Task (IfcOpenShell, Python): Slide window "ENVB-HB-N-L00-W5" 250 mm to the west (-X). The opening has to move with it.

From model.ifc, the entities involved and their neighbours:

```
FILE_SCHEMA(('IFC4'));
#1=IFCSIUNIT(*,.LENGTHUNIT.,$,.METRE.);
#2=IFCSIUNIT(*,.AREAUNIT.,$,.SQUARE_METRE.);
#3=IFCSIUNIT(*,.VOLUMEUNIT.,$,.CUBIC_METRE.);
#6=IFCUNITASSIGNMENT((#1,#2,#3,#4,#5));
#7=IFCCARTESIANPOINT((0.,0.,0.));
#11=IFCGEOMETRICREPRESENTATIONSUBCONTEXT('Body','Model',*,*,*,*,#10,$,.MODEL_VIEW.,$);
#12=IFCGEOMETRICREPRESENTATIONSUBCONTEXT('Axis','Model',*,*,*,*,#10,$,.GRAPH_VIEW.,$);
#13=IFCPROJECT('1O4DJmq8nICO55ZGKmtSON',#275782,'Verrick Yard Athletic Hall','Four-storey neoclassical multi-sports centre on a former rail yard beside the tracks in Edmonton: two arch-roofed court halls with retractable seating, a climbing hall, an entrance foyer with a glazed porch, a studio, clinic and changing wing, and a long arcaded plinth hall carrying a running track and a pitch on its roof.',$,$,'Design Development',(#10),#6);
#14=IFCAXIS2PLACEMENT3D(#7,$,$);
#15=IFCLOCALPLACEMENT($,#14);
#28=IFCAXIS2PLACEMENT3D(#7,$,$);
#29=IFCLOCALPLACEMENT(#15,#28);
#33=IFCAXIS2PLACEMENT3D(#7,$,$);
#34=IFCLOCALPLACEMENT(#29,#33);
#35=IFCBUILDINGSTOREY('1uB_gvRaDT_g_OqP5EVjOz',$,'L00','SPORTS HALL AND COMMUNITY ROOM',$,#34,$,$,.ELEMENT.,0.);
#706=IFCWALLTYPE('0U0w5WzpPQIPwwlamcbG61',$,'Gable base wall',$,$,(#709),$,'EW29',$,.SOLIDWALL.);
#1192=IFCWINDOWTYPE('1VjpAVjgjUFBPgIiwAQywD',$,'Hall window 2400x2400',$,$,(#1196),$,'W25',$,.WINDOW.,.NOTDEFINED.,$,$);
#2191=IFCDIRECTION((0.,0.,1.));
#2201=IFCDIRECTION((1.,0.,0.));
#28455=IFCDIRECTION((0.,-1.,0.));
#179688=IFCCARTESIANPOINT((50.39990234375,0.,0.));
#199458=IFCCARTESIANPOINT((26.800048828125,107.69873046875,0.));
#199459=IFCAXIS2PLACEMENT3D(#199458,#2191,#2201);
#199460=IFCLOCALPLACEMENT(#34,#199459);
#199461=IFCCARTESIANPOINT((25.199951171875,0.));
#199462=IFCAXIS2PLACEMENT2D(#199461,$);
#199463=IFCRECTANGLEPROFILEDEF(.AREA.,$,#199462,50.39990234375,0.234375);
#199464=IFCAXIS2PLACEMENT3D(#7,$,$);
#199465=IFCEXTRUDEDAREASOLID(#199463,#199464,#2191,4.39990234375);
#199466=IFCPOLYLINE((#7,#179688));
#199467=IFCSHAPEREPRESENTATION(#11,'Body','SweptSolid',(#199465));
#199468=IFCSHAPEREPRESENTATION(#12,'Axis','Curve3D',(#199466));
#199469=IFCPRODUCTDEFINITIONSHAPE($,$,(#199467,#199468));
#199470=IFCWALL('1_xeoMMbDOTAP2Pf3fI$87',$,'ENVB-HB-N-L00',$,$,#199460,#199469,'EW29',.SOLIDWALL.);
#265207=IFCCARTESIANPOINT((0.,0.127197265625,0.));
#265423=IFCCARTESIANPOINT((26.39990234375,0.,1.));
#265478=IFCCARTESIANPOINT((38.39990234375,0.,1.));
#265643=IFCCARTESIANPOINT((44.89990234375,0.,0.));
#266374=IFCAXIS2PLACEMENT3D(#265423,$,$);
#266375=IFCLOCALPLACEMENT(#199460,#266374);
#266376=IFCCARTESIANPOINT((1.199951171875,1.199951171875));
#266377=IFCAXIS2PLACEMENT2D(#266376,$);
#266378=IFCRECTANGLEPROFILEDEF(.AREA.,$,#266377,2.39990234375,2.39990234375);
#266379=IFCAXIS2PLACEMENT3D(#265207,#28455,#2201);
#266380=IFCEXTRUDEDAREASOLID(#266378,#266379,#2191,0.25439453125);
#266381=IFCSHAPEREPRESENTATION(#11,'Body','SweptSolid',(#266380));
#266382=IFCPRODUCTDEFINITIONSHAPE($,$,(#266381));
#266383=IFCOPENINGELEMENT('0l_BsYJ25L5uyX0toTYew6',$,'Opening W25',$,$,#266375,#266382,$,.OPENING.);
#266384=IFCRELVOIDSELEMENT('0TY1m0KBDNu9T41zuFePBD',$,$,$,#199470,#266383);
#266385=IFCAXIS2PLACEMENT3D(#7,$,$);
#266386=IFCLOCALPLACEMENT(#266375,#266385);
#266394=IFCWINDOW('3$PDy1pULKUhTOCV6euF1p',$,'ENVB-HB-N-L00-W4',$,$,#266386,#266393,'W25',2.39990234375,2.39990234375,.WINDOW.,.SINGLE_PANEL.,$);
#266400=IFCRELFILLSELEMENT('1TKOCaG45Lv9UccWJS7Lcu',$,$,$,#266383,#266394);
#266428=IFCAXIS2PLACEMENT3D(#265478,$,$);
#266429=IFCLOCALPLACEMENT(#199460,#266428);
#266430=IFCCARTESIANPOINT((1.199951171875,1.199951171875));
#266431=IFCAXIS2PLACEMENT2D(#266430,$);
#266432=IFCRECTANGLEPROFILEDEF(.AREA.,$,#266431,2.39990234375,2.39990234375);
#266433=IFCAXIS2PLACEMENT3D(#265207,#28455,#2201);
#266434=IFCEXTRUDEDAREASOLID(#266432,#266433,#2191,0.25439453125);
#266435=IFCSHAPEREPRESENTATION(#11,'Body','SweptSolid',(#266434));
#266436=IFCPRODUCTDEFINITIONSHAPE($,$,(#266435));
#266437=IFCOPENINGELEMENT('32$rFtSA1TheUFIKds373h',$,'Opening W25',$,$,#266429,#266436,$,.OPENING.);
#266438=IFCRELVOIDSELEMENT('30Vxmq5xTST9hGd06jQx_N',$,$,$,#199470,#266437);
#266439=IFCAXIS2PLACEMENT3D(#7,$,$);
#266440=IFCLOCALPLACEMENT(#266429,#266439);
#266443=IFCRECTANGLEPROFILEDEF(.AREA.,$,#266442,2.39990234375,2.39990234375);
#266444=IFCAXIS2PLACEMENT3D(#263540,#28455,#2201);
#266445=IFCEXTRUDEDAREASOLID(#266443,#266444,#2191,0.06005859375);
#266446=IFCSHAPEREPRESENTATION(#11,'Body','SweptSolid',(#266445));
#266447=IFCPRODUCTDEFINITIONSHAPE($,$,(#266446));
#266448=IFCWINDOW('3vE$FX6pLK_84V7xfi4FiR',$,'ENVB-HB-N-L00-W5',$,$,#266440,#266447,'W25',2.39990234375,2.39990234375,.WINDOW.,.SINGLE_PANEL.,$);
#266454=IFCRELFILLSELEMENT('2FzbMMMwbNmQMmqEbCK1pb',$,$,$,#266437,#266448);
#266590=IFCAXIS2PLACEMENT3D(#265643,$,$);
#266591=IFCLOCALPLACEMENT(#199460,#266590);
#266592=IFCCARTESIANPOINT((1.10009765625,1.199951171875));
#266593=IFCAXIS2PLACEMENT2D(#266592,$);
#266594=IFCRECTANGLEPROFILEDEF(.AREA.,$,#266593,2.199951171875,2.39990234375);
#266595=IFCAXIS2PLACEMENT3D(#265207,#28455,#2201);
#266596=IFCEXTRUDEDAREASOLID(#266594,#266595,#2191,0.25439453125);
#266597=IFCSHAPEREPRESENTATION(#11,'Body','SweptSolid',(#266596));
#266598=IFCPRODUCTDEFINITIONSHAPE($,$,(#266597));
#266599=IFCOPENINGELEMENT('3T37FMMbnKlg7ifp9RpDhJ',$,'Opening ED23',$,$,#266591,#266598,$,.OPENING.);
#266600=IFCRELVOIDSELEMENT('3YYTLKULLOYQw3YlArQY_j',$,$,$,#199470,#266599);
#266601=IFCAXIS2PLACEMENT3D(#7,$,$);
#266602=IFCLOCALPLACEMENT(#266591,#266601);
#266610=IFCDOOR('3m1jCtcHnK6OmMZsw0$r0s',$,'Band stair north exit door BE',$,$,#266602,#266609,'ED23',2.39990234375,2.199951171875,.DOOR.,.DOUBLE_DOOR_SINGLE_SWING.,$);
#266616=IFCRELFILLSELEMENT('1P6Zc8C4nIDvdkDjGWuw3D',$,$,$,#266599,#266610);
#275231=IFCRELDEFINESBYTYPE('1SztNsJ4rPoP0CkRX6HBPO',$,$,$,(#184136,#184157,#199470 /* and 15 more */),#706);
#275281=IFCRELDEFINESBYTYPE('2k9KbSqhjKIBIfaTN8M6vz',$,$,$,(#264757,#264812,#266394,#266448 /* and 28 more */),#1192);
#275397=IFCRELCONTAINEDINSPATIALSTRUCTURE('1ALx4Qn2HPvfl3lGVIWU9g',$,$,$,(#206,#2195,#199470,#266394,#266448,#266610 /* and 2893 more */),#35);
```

```python
import ifcopenshell
import ifcopenshell.api.geometry
import ifcopenshell.util.placement
import ifcopenshell.util.unit

model = ifcopenshell.open("model.ifc")
unit_scale = ifcopenshell.util.unit.calculate_unit_scale(model)

window = model.by_guid("3vE$FX6pLK_84V7xfi4FiR")
opening = window.FillsVoids[0].RelatingOpeningElement
wall = opening.VoidsElements[0].RelatingBuildingElement

wall_matrix = ifcopenshell.util.placement.get_local_placement(wall.ObjectPlacement)
shift = wall_matrix[:3, 0] * -0.25 / unit_scale
before = ifcopenshell.util.placement.get_local_placement(window.ObjectPlacement)[:3, 3].copy()

# The window is placed relative to its opening, so it follows when the opening moves.
matrix = ifcopenshell.util.placement.get_local_placement(opening.ObjectPlacement)
matrix[:3, 3] += shift
ifcopenshell.api.geometry.edit_object_placement(
    model, product=opening, matrix=matrix, is_si=False, should_transform_children=True
)

after = ifcopenshell.util.placement.get_local_placement(window.ObjectPlacement)[:3, 3]
print("window moved by", (after - before).round(3) + 0.0)

model.write("model_rev.ifc")
```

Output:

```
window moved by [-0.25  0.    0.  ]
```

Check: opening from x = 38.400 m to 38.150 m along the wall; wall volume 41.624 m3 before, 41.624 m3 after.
